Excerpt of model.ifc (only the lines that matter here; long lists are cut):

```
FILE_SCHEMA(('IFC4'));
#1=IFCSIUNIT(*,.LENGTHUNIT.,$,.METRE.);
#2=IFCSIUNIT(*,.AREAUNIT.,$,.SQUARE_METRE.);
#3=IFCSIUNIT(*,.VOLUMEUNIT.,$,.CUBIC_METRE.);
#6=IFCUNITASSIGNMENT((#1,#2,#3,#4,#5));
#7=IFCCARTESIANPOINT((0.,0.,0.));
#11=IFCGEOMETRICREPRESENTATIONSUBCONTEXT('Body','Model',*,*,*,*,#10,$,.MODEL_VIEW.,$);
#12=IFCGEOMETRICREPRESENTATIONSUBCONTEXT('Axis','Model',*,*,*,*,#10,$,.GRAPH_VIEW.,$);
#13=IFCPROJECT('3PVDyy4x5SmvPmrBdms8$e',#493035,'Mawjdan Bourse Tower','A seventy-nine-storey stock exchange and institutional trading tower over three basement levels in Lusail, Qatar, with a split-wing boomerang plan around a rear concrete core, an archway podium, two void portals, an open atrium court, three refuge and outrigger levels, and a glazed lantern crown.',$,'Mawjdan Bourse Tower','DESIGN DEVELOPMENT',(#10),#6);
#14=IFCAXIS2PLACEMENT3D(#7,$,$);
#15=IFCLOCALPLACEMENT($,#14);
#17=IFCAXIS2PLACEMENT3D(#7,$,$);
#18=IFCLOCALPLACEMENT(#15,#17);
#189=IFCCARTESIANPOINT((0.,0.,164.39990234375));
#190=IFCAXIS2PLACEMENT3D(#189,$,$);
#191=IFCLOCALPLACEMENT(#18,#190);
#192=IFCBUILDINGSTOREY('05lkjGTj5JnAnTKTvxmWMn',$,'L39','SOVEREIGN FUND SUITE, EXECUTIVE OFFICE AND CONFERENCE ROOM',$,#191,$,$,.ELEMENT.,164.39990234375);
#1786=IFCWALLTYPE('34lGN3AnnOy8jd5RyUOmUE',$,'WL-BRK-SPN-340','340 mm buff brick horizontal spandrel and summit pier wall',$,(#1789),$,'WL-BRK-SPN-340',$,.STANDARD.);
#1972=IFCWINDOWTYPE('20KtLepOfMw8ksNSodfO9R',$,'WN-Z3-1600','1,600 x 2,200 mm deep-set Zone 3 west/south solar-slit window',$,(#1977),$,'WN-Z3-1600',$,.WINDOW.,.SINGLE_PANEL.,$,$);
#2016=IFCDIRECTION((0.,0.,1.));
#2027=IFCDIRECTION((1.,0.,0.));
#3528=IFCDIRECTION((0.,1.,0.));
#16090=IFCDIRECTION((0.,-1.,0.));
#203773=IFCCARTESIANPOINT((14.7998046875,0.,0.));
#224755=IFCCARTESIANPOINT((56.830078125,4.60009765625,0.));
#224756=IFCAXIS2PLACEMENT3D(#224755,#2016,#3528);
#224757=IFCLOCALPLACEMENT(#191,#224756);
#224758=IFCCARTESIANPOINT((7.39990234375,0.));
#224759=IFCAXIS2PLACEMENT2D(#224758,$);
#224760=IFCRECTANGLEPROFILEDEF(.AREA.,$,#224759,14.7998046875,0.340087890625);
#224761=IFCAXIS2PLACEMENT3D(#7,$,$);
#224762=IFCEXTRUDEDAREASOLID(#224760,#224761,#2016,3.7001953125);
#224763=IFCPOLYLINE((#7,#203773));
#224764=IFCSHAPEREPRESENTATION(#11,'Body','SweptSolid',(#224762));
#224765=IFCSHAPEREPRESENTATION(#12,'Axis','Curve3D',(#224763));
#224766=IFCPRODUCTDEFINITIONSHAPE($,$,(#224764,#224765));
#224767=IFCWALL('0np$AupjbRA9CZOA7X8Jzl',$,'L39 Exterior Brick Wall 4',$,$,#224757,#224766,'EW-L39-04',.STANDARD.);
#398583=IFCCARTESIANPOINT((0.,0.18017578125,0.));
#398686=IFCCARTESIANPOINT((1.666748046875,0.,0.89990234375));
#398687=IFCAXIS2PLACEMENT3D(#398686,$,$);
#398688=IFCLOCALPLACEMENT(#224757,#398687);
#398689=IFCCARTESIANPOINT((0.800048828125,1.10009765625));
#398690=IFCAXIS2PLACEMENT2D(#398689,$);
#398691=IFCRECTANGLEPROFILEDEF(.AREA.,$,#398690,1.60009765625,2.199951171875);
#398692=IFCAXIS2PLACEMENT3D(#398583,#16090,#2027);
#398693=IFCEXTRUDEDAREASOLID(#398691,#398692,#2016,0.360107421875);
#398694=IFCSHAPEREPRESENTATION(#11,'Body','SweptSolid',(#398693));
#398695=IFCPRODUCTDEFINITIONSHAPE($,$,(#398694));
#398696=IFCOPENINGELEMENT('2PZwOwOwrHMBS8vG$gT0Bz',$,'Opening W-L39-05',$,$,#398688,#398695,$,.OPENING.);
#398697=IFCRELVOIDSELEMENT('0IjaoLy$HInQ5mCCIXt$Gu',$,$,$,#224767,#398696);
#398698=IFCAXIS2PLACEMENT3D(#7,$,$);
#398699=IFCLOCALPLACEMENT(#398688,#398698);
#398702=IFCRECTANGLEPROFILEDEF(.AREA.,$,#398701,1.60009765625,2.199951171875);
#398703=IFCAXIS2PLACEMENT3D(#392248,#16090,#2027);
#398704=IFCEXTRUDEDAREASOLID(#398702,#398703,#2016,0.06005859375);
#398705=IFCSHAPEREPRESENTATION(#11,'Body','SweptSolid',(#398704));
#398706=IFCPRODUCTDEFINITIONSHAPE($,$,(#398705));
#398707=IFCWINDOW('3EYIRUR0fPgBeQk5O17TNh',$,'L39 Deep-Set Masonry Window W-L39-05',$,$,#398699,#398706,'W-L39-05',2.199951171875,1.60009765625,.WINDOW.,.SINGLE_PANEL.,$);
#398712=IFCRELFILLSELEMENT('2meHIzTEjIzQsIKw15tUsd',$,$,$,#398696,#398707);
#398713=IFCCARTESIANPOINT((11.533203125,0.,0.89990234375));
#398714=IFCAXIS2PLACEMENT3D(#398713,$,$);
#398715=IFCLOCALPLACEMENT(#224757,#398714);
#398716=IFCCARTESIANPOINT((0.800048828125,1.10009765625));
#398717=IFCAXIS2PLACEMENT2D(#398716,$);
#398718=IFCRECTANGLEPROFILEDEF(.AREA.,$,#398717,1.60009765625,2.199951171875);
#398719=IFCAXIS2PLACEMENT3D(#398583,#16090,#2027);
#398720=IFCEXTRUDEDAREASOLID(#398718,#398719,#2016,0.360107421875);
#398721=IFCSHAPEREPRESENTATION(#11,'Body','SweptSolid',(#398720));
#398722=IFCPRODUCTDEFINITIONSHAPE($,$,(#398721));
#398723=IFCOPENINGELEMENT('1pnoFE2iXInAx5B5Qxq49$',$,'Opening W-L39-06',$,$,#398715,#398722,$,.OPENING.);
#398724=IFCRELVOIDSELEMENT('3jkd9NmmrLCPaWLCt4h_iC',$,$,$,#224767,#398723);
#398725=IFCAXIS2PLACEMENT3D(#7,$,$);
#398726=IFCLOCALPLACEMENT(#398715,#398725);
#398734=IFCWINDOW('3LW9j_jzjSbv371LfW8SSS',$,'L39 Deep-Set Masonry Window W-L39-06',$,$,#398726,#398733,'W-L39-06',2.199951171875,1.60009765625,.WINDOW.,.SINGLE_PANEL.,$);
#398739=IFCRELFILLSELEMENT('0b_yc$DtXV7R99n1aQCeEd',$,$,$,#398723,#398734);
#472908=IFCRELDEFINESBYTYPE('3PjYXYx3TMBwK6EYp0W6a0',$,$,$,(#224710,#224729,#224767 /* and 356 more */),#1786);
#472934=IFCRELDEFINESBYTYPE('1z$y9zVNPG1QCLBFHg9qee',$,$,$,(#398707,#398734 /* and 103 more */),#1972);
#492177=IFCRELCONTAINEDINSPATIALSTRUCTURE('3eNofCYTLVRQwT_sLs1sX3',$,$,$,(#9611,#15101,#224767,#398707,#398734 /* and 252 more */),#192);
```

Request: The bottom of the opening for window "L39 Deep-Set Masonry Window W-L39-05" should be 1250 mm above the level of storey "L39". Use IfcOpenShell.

```python
import numpy as np
import ifcopenshell
import ifcopenshell.api.geometry
import ifcopenshell.geom
import ifcopenshell.util.element
import ifcopenshell.util.placement
import ifcopenshell.util.shape
import ifcopenshell.util.unit

model = ifcopenshell.open("model.ifc")
unit_scale = ifcopenshell.util.unit.calculate_unit_scale(model)

window = model.by_guid("3EYIRUR0fPgBeQk5O17TNh")
opening = window.FillsVoids[0].RelatingOpeningElement
storey = ifcopenshell.util.element.get_container(window, ifc_class="IfcBuildingStorey")
level = ifcopenshell.util.placement.get_local_placement(storey.ObjectPlacement)[2, 3]

# The opening's origin need not be at the sill, so measure its lowest point.
shape = ifcopenshell.geom.create_shape(ifcopenshell.geom.settings(), opening)
bottom = ifcopenshell.util.shape.get_shape_bottom_elevation(shape, shape.geometry) / unit_scale
dz = level + 1.25 / unit_scale - bottom

shift = np.array([0.0, 0.0, dz])
# The window is placed relative to its opening, so it follows when the opening moves.
matrix = ifcopenshell.util.placement.get_local_placement(opening.ObjectPlacement)
matrix[:3, 3] += shift
ifcopenshell.api.geometry.edit_object_placement(
    model, product=opening, matrix=matrix, is_si=False, should_transform_children=True
)

print(f"moved by {dz * unit_scale:+.3f} m")

model.write("model_v2.ifc")
```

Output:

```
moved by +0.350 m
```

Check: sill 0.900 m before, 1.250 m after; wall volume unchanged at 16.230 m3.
